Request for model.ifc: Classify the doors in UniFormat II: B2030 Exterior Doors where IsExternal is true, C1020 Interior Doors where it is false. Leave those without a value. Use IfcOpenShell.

First a look at what the model holds.

```python
import ifcopenshell
import ifcopenshell.util.element

model = ifcopenshell.open("model.ifc")
print(model.schema)
print("classifications:", [c.Name for c in model.by_type("IfcClassification")])
values = [ifcopenshell.util.element.get_pset(e, "Pset_DoorCommon", "IsExternal") for e in model.by_type("IfcDoor")]
for value in (True, False, None):
    print("IsExternal", value, values.count(value))
```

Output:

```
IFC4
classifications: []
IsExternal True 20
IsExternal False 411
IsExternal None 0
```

```python
import ifcopenshell
import ifcopenshell.api.classification
import ifcopenshell.util.element

model = ifcopenshell.open("model.ifc")

system = ifcopenshell.api.classification.add_classification(model, classification="UniFormat II")

doors = model.by_type("IfcDoor")
external = {e: ifcopenshell.util.element.get_pset(e, "Pset_DoorCommon", "IsExternal") for e in doors}
for flag, code, name in ((True, "B2030", "Exterior Doors"), (False, "C1020", "Interior Doors")):
    products = [e for e in doors if external[e] is flag]
    ifcopenshell.api.classification.add_reference(
        model, products=products, classification=system, identification=code, name=name
    )
    print(code, len(products))

model.write("model_v2.ifc")
```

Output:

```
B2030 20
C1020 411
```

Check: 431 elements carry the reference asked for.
